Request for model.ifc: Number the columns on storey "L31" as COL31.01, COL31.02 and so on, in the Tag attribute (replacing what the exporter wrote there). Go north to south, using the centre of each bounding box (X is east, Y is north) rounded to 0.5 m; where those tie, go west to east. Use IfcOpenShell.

First a look at what the model holds.

```python
import ifcopenshell
import ifcopenshell.util.element
import ifcopenshell.util.placement

model = ifcopenshell.open("model.ifc")
print(model.schema)
storey = next(s for s in model.by_type("IfcBuildingStorey") if s.Name == "L31")
columns = [e for e in ifcopenshell.util.element.get_decomposition(storey) if e.is_a("IfcColumn")]
for e in sorted(columns, key=lambda e: e.id()):
    origin = ifcopenshell.util.placement.get_local_placement(e.ObjectPlacement)[:3, 3]
    print(e.id(), e.Tag, e.Name, origin.round(2) + 0.0, sep=" | ")
```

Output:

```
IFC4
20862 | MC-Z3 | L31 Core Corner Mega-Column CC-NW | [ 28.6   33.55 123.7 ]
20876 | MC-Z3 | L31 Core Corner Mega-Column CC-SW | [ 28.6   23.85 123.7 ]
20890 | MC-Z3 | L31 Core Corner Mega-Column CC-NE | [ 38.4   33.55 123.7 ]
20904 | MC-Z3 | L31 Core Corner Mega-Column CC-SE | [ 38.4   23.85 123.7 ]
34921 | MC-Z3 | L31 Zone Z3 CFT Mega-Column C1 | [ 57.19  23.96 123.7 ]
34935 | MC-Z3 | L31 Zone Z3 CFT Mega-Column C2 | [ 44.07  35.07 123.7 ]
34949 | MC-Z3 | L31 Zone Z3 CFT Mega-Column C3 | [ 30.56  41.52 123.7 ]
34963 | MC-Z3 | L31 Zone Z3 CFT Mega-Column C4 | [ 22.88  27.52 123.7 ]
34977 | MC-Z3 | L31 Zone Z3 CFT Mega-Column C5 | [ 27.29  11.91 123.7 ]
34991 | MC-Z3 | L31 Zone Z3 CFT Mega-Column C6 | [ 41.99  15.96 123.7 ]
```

```python
import ifcopenshell
import ifcopenshell.geom
import ifcopenshell.util.element
import ifcopenshell.util.shape

model = ifcopenshell.open("model.ifc")
settings = ifcopenshell.geom.settings()
settings.set("use-world-coords", True)


def centre(element):
    shape = ifcopenshell.geom.create_shape(settings, element)
    return ifcopenshell.util.shape.get_bbox_centroid(shape.geometry)


storey = next(s for s in model.by_type("IfcBuildingStorey") if s.Name == "L31")
columns = [e for e in ifcopenshell.util.element.get_decomposition(storey) if e.is_a("IfcColumn")]

# Insertion points can sit at a corner or the storey origin, so sort by the geometry (in metres).
centres = {e: centre(e) for e in columns}
columns.sort(key=lambda e: (-round(centres[e][1] / 0.5), centres[e][0]))

for i, e in enumerate(columns, start=1):
    number = f"COL31.{i:02d}"
    e.Tag = number
    print(e.id(), number)

model.write("model_rev.ifc")
```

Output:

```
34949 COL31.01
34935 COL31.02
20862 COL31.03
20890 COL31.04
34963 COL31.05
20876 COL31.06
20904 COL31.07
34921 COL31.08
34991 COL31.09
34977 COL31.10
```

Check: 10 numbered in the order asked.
